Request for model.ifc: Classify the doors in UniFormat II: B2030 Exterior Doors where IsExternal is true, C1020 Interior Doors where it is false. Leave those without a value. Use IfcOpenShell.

First a look at what the model holds.

```python
import ifcopenshell
import ifcopenshell.util.element

model = ifcopenshell.open("model.ifc")
print(model.schema)
print("classifications:", [c.Name for c in model.by_type("IfcClassification")])
values = [ifcopenshell.util.element.get_pset(e, "Pset_DoorCommon", "IsExternal") for e in model.by_type("IfcDoor")]
for value in (True, False, None):
    print("IsExternal", value, values.count(value))
```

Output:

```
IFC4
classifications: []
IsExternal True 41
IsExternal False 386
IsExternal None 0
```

```python
import ifcopenshell
import ifcopenshell.api.classification
import ifcopenshell.util.element

model = ifcopenshell.open("model.ifc")

system = ifcopenshell.api.classification.add_classification(model, classification="UniFormat II")

doors = model.by_type("IfcDoor")
external = {e: ifcopenshell.util.element.get_pset(e, "Pset_DoorCommon", "IsExternal") for e in doors}
for flag, code, name in ((True, "B2030", "Exterior Doors"), (False, "C1020", "Interior Doors")):
    products = [e for e in doors if external[e] is flag]
    ifcopenshell.api.classification.add_reference(
        model, products=products, classification=system, identification=code, name=name
    )
    print(code, len(products))

model.write("model-out.ifc")
```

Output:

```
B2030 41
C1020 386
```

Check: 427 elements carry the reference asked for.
